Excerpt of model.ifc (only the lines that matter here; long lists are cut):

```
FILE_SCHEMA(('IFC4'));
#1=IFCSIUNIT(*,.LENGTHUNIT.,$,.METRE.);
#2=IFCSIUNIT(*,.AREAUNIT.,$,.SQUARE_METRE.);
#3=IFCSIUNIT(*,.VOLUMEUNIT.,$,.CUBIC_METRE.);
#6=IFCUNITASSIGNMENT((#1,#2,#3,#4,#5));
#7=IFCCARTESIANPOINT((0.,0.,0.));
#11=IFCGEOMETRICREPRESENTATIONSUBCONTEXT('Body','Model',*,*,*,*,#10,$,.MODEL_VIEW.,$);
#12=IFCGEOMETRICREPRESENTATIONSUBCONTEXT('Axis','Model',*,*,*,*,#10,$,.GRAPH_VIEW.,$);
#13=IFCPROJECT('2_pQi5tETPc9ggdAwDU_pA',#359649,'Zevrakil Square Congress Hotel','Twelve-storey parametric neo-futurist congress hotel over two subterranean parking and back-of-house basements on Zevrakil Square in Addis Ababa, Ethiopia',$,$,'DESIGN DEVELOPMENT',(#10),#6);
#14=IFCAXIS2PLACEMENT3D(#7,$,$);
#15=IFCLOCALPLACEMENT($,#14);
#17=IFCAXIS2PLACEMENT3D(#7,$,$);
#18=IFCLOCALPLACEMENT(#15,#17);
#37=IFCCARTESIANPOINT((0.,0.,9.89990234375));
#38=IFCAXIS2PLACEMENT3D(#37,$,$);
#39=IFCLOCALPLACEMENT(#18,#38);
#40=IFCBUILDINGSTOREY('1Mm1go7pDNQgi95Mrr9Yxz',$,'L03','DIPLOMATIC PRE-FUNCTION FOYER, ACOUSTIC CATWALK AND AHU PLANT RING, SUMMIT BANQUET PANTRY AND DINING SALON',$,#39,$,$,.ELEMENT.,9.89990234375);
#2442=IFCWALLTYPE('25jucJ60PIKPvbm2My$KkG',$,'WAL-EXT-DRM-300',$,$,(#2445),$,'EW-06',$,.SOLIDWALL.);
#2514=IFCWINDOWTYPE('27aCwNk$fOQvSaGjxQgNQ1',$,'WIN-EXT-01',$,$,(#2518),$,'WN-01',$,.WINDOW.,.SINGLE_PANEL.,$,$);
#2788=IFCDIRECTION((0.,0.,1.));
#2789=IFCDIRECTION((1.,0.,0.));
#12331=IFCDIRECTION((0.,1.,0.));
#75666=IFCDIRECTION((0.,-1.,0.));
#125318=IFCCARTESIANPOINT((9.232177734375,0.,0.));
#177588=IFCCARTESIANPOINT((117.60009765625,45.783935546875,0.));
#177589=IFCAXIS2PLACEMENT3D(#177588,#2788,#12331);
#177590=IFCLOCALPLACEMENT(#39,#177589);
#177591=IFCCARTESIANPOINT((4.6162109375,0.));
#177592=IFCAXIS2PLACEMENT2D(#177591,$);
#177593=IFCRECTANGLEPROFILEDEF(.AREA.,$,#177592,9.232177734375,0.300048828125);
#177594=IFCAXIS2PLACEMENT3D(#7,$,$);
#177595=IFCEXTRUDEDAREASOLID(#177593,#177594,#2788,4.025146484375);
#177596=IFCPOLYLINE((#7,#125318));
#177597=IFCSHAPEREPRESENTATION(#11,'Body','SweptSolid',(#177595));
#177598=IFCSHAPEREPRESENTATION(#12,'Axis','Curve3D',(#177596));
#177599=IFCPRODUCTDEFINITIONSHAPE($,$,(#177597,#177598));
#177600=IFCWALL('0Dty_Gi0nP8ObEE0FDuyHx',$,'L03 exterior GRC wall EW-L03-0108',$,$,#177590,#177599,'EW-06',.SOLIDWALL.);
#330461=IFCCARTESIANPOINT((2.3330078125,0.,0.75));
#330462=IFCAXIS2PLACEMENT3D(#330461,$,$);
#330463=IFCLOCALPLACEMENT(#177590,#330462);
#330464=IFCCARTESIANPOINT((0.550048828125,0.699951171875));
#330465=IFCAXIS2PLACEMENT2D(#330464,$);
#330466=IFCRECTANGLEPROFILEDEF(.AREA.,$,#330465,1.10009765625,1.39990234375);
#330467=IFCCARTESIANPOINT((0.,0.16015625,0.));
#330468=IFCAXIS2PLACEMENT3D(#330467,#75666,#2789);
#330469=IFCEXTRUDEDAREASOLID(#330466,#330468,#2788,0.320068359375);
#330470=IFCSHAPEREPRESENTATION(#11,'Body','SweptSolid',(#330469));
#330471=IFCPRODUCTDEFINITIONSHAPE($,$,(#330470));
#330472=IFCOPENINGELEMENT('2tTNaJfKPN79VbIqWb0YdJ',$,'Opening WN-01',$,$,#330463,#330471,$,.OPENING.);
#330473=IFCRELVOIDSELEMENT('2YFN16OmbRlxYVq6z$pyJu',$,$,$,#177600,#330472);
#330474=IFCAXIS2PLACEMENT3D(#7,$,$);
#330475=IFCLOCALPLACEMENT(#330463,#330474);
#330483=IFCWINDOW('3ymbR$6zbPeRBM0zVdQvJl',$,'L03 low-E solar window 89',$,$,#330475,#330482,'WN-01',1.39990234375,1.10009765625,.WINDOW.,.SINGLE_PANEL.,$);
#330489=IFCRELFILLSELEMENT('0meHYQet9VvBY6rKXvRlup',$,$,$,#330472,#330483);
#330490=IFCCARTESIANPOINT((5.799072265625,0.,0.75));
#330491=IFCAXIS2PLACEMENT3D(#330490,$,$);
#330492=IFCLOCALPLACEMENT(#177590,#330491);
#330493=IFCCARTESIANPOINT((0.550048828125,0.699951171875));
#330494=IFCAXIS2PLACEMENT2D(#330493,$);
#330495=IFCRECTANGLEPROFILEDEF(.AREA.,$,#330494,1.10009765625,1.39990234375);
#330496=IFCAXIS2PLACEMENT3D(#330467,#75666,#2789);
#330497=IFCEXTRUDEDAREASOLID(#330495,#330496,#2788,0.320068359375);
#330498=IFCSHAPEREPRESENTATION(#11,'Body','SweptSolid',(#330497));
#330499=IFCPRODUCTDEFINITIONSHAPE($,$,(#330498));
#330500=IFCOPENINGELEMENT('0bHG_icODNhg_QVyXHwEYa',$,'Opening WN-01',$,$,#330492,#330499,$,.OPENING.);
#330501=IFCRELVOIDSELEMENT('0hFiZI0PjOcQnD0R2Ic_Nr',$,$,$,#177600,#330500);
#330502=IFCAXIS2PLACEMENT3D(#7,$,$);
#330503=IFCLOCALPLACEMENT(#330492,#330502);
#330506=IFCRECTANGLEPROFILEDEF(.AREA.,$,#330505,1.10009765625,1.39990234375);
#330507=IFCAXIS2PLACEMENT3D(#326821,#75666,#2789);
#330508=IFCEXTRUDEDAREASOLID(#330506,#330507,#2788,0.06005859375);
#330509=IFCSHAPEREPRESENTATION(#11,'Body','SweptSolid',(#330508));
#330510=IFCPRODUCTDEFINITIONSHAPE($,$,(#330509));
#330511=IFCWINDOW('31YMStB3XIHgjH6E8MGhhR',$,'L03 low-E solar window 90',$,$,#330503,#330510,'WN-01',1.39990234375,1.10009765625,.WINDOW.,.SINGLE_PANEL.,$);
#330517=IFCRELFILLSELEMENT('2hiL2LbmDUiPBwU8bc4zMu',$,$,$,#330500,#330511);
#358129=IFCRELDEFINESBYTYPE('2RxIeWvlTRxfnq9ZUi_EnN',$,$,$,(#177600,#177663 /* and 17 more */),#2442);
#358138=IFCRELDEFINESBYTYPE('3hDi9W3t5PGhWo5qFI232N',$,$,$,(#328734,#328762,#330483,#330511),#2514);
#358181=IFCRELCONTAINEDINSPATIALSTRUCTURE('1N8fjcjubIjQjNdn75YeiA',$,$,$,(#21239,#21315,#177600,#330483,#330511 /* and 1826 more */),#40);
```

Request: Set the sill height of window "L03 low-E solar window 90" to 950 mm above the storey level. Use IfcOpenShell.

```python
import numpy as np
import ifcopenshell
import ifcopenshell.api.geometry
import ifcopenshell.geom
import ifcopenshell.util.element
import ifcopenshell.util.placement
import ifcopenshell.util.shape
import ifcopenshell.util.unit

model = ifcopenshell.open("model.ifc")
unit_scale = ifcopenshell.util.unit.calculate_unit_scale(model)

window = model.by_guid("31YMStB3XIHgjH6E8MGhhR")
opening = window.FillsVoids[0].RelatingOpeningElement
storey = ifcopenshell.util.element.get_container(window, ifc_class="IfcBuildingStorey")
level = ifcopenshell.util.placement.get_local_placement(storey.ObjectPlacement)[2, 3]

# The opening's origin need not be at the sill, so measure its lowest point.
shape = ifcopenshell.geom.create_shape(ifcopenshell.geom.settings(), opening)
bottom = ifcopenshell.util.shape.get_shape_bottom_elevation(shape, shape.geometry) / unit_scale
dz = level + 0.95 / unit_scale - bottom

shift = np.array([0.0, 0.0, dz])
# The window is placed relative to its opening, so it follows when the opening moves.
matrix = ifcopenshell.util.placement.get_local_placement(opening.ObjectPlacement)
matrix[:3, 3] += shift
ifcopenshell.api.geometry.edit_object_placement(
    model, product=opening, matrix=matrix, is_si=False, should_transform_children=True
)

print(f"moved by {dz * unit_scale:+.3f} m")

model.write("model_v2.ifc")
```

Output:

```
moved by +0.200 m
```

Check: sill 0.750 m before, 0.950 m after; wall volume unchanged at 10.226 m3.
